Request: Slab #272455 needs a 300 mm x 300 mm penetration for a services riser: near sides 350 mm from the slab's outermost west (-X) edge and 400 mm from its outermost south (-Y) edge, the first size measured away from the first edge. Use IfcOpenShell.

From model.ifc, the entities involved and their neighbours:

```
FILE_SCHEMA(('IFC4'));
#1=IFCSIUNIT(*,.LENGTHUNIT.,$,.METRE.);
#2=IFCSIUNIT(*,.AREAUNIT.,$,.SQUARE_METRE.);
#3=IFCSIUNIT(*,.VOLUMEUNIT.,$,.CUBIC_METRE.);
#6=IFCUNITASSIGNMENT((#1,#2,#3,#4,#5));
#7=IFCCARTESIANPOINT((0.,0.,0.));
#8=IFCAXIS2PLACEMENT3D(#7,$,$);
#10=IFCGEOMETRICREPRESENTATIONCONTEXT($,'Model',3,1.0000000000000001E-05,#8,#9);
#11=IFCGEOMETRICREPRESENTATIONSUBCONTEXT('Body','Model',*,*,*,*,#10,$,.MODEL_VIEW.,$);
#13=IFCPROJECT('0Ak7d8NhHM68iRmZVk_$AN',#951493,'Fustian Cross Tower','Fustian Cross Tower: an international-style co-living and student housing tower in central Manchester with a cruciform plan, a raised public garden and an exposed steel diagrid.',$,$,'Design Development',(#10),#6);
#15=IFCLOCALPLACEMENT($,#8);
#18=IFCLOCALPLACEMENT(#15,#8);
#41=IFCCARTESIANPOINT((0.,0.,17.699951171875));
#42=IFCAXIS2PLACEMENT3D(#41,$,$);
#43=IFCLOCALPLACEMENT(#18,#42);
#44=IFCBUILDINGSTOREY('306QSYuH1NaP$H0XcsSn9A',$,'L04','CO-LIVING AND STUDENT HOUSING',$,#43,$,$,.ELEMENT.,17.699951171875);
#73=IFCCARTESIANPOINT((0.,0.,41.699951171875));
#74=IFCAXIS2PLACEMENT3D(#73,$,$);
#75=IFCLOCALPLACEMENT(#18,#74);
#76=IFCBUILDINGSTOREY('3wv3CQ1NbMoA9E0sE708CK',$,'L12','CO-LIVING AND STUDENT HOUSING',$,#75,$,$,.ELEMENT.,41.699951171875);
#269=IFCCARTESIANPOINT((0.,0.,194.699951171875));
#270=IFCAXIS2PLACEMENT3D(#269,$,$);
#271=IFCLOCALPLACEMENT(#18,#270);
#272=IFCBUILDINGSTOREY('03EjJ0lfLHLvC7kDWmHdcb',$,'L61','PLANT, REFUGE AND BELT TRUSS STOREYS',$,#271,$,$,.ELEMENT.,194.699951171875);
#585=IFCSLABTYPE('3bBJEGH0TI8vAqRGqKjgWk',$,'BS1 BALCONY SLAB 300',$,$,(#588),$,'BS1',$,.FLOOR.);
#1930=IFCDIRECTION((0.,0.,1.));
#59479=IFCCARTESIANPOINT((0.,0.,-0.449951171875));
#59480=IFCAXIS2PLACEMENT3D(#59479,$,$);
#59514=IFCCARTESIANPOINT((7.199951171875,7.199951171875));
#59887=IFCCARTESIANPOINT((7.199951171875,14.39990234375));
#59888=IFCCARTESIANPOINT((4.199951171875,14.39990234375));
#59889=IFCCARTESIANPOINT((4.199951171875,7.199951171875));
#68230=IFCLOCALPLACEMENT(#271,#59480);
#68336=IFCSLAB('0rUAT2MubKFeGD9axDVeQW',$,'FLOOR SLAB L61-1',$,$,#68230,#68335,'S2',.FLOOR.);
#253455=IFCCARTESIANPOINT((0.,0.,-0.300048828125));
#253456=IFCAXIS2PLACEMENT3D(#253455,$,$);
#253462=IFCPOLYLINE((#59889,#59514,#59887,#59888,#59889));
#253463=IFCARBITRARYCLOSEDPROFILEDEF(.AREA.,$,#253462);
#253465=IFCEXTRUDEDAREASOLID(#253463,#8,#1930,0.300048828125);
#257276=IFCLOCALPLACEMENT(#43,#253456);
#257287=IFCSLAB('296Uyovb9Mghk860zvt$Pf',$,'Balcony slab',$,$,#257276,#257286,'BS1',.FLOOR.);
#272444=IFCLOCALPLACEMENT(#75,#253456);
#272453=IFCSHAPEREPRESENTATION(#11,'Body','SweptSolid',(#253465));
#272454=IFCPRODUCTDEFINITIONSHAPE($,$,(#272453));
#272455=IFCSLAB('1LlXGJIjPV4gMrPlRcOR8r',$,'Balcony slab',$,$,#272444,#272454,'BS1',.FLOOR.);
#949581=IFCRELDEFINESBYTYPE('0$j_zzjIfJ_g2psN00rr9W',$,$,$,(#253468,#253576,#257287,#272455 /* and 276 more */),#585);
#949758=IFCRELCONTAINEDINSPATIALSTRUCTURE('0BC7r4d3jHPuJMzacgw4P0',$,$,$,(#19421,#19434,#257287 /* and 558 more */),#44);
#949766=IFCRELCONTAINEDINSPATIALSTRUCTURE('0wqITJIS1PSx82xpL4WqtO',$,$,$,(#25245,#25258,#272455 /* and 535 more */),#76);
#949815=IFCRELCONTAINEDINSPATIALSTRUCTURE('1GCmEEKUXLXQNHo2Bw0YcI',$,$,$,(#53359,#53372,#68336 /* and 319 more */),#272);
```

```python
import numpy as np
import ifcopenshell
import ifcopenshell.api.feature
import ifcopenshell.api.geometry
import ifcopenshell.api.root
import ifcopenshell.geom
import ifcopenshell.util.placement
import ifcopenshell.util.representation
import ifcopenshell.util.shape
import ifcopenshell.util.unit

model = ifcopenshell.open("model.ifc")
unit_scale = ifcopenshell.util.unit.calculate_unit_scale(model)
settings = ifcopenshell.geom.settings()


def volume(element):
    """Net volume in cubic metres, openings subtracted."""
    shape = ifcopenshell.geom.create_shape(settings, element)
    return ifcopenshell.util.shape.get_volume(shape.geometry)


slab = model.by_guid("1LlXGJIjPV4gMrPlRcOR8r")
before = volume(slab)

# Extent in the slab's own axes, in metres. The edges named are its -X and -Y sides.
slab_shape = ifcopenshell.geom.create_shape(settings, slab)
vertices = ifcopenshell.util.shape.get_vertices(slab_shape.geometry)
x_min, y_min, bottom = vertices.min(axis=0)
top = vertices[:, 2].max()

opening = ifcopenshell.api.root.create_entity(model, ifc_class="IfcOpeningElement", name="Services riser opening", predefined_type="OPENING")
context = ifcopenshell.util.representation.get_context(model, "Model", "Body", "MODEL_VIEW")
width, depth = 0.3, 0.3
outline = [(0.0, 0.0), (width, 0.0), (width, depth), (0.0, depth), (0.0, 0.0)]
# Overshoot both faces by 50 mm so the cut is clean.
shape = ifcopenshell.api.geometry.add_slab_representation(
    model, context=context, depth=top - bottom + 0.1, polyline=outline
)
ifcopenshell.api.geometry.assign_representation(model, product=opening, representation=shape)

matrix = ifcopenshell.util.placement.get_local_placement(slab.ObjectPlacement)
matrix[:, 3] = matrix @ np.append(np.array([x_min + 0.35, y_min + 0.4, bottom - 0.05]) / unit_scale, 1.0)
ifcopenshell.api.geometry.edit_object_placement(model, product=opening, matrix=matrix, is_si=False)
ifcopenshell.api.feature.add_feature(model, feature=opening, element=slab)

after = volume(slab)

print(f"slab volume {before:.3f} -> {after:.3f} m3")

model.write("model_v2.ifc")
```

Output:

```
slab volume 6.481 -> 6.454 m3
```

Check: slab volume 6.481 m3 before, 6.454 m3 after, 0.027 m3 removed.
